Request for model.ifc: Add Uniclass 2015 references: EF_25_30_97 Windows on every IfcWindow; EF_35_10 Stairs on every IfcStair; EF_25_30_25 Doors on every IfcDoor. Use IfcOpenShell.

First a look at what the model holds.

```python
import ifcopenshell

model = ifcopenshell.open("model.ifc")
print(model.schema)
print("classifications:", [c.Name for c in model.by_type("IfcClassification")])
for ifc_class in ("IfcDoor", "IfcRoof", "IfcStair", "IfcWall", "IfcWindow"):
    print(ifc_class, len(model.by_type(ifc_class)))
```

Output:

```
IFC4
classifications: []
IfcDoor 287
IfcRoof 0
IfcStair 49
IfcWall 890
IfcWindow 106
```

```python
import ifcopenshell
import ifcopenshell.api.classification

model = ifcopenshell.open("model.ifc")

system = ifcopenshell.api.classification.add_classification(model, classification="Uniclass 2015")

codes = {
    "IfcWindow": ("EF_25_30_97", "Windows"),
    "IfcStair": ("EF_35_10", "Stairs"),
    "IfcDoor": ("EF_25_30_25", "Doors"),
}
for ifc_class, (code, name) in codes.items():
    products = model.by_type(ifc_class)
    ifcopenshell.api.classification.add_reference(
        model, products=products, classification=system, identification=code, name=name
    )
    print(code, len(products))

model.write("model_updated.ifc")
```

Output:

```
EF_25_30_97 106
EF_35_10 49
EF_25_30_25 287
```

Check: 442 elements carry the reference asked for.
